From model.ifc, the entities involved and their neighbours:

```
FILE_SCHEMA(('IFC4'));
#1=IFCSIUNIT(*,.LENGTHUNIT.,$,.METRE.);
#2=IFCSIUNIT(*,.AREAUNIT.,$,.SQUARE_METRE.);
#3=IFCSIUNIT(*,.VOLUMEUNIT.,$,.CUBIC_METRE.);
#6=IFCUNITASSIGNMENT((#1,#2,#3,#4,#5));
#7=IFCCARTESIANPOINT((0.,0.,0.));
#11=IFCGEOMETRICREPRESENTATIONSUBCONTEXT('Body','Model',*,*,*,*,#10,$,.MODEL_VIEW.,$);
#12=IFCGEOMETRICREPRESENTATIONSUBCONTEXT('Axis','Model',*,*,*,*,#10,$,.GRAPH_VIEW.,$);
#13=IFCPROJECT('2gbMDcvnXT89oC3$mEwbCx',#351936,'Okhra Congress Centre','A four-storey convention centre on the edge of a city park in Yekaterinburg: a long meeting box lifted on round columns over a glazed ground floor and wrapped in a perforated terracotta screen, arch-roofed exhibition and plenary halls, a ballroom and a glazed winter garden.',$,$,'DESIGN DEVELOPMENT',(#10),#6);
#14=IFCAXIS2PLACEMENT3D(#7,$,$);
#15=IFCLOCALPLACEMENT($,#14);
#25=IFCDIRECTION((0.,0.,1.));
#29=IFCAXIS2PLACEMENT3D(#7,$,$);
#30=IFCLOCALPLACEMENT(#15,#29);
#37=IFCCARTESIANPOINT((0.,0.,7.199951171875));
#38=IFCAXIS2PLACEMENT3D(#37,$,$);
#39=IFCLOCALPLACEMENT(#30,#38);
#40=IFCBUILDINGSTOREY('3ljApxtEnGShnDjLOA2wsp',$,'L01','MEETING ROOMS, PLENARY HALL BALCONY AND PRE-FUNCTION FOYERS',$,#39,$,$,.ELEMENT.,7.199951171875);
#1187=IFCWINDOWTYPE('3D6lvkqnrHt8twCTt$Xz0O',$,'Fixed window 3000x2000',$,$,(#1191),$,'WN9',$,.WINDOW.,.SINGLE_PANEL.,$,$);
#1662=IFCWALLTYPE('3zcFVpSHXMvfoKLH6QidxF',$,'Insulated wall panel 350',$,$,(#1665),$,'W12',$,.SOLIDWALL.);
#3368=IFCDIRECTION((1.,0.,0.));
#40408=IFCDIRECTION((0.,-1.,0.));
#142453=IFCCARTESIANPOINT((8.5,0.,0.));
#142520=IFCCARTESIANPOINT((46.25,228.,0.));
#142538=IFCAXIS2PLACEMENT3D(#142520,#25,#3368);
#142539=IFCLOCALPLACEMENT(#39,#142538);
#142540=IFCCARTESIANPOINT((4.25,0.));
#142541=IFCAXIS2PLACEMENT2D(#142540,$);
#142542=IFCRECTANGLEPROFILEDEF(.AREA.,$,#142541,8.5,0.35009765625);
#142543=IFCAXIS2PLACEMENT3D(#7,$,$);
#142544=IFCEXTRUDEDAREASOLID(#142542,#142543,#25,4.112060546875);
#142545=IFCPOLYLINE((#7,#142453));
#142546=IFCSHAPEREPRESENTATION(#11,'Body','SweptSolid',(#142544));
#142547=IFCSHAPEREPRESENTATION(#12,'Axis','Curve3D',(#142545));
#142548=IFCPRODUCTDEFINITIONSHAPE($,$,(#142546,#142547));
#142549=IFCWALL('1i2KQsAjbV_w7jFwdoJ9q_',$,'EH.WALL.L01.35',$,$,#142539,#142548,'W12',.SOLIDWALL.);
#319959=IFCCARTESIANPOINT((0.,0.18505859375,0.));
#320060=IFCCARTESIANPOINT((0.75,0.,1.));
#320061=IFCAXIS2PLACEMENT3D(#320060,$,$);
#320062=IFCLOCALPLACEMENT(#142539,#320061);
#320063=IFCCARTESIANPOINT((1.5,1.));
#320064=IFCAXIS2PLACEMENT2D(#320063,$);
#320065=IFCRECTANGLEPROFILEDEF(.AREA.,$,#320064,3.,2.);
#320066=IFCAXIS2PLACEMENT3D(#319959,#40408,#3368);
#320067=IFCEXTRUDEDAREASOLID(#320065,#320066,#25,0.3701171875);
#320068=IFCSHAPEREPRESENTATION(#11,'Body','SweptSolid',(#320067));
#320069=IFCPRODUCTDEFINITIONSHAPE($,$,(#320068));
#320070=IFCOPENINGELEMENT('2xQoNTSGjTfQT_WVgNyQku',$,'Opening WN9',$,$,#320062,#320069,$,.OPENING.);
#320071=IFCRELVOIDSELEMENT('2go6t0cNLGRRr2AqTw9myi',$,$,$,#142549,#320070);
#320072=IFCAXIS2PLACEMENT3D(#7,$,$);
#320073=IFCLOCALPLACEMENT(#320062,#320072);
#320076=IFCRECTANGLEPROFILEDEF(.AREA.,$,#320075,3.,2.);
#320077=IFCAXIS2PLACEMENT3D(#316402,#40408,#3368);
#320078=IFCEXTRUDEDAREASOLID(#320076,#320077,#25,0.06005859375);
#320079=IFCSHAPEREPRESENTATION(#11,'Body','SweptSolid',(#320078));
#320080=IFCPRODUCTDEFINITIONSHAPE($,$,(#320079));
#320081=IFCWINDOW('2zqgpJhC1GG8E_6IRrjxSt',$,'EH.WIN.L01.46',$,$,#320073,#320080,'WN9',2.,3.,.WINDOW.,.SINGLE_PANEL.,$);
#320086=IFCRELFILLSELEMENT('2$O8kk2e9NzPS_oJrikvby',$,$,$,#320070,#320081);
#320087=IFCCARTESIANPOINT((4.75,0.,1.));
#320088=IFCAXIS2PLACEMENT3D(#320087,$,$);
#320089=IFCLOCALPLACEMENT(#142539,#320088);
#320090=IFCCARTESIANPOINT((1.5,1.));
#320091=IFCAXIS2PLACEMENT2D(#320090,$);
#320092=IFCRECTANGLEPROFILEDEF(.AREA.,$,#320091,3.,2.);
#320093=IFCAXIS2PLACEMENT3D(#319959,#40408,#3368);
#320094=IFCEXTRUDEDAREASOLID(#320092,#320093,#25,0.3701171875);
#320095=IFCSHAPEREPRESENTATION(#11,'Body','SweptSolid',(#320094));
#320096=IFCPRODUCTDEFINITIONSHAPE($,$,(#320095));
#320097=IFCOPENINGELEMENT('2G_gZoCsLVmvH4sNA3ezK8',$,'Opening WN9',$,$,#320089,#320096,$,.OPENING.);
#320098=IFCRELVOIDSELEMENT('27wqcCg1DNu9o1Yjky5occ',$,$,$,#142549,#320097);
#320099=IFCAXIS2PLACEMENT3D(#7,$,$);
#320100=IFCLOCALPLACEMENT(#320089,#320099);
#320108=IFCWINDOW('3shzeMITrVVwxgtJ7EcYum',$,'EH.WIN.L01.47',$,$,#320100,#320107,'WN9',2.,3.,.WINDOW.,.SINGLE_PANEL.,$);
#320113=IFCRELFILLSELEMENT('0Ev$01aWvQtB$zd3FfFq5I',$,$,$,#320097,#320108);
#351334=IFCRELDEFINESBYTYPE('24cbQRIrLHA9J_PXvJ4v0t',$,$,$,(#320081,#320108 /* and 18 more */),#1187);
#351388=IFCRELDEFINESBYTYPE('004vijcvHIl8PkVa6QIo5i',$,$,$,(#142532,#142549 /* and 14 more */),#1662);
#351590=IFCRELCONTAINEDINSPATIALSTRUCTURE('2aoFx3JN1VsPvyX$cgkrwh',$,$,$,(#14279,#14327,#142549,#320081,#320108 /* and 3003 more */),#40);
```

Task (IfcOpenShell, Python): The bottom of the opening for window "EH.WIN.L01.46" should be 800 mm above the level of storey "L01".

```python
import numpy as np
import ifcopenshell
import ifcopenshell.api.geometry
import ifcopenshell.geom
import ifcopenshell.util.element
import ifcopenshell.util.placement
import ifcopenshell.util.shape
import ifcopenshell.util.unit

model = ifcopenshell.open("model.ifc")
unit_scale = ifcopenshell.util.unit.calculate_unit_scale(model)

window = model.by_id(320081)
opening = window.FillsVoids[0].RelatingOpeningElement
storey = ifcopenshell.util.element.get_container(window, ifc_class="IfcBuildingStorey")
level = ifcopenshell.util.placement.get_local_placement(storey.ObjectPlacement)[2, 3]

# The opening's origin need not be at the sill, so measure its lowest point.
shape = ifcopenshell.geom.create_shape(ifcopenshell.geom.settings(), opening)
bottom = ifcopenshell.util.shape.get_shape_bottom_elevation(shape, shape.geometry) / unit_scale
dz = level + 0.8 / unit_scale - bottom

shift = np.array([0.0, 0.0, dz])
# The window is placed relative to its opening, so it follows when the opening moves.
matrix = ifcopenshell.util.placement.get_local_placement(opening.ObjectPlacement)
matrix[:3, 3] += shift
ifcopenshell.api.geometry.edit_object_placement(
    model, product=opening, matrix=matrix, is_si=False, should_transform_children=True
)

print(f"moved by {dz * unit_scale:+.3f} m")

model.write("model-out.ifc")
```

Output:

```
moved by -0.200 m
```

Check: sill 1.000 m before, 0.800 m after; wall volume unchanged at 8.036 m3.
